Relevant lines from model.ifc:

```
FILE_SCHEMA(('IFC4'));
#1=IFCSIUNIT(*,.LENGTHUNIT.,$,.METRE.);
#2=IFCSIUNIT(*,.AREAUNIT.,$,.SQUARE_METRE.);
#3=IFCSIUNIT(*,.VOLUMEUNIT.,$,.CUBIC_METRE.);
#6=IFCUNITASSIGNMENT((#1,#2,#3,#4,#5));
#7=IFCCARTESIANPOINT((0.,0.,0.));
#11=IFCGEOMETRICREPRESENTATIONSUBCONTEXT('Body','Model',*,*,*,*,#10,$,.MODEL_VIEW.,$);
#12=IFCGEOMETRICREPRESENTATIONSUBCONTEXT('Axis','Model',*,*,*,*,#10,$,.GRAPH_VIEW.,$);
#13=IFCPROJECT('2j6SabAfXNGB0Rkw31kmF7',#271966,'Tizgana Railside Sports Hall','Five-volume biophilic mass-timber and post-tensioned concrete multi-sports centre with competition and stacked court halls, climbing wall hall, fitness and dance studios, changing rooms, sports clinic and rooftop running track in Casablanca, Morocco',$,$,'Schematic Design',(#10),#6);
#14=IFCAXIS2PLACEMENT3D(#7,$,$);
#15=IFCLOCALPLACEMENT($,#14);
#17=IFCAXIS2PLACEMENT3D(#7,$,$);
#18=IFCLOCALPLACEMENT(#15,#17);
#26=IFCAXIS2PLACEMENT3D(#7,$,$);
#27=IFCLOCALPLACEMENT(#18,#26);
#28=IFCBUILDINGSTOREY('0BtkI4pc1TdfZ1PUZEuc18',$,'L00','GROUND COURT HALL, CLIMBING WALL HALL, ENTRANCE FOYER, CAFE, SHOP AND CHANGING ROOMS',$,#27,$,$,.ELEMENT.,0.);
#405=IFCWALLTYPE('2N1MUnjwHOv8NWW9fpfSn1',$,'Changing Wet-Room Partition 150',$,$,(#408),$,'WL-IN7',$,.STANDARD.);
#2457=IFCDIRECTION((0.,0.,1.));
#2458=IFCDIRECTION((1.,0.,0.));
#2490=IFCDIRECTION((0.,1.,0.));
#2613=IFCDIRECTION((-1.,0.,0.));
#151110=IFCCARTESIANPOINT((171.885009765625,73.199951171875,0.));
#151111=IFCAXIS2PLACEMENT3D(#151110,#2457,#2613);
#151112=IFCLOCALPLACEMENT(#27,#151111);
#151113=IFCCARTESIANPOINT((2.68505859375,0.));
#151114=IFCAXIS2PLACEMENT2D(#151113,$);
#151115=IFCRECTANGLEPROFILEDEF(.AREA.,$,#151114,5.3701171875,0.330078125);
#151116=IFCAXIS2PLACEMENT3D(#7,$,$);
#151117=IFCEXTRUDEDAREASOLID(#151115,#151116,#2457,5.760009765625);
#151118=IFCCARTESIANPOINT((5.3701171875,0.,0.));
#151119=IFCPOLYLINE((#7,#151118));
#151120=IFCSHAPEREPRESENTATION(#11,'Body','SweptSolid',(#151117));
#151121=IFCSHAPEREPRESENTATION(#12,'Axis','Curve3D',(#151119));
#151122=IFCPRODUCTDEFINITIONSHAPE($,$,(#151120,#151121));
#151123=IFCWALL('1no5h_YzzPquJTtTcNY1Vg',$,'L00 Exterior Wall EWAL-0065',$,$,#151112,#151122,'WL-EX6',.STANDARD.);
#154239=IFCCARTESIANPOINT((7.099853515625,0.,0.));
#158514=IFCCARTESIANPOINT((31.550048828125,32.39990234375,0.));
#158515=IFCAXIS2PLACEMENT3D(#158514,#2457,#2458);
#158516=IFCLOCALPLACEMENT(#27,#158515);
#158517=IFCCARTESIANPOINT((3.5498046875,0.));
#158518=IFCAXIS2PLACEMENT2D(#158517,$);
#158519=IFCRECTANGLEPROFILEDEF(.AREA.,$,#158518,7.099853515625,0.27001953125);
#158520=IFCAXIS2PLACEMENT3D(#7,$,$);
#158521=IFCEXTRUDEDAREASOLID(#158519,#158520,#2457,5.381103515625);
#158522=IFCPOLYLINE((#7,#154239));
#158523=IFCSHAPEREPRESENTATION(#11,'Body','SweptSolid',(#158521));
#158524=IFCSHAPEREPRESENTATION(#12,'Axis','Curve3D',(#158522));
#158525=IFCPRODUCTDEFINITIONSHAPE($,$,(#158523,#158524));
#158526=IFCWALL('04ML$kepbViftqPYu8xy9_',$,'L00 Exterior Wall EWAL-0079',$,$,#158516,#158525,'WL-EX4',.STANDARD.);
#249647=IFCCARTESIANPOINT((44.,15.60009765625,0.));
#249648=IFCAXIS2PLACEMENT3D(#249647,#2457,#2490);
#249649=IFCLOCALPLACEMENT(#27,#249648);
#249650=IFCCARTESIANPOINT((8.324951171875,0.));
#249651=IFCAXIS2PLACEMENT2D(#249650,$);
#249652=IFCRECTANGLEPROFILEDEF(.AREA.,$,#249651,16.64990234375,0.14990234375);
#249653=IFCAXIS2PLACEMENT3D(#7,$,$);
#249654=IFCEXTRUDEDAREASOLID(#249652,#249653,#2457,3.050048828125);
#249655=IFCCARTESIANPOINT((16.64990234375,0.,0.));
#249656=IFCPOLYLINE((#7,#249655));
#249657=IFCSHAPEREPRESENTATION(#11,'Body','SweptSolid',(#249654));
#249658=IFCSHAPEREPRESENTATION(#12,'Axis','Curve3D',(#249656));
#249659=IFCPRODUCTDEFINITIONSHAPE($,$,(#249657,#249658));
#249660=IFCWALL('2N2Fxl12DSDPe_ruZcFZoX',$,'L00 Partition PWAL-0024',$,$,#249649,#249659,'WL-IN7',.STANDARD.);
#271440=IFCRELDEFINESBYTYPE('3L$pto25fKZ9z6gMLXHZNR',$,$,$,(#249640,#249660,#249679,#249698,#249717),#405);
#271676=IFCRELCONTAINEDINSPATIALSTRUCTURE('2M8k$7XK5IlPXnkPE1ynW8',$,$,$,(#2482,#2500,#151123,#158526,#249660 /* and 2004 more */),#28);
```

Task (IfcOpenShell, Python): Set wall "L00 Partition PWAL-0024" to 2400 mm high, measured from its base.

```python
import ifcopenshell
import ifcopenshell.geom
import ifcopenshell.util.representation
import ifcopenshell.util.shape
import ifcopenshell.util.unit

model = ifcopenshell.open("model.ifc")
unit_scale = ifcopenshell.util.unit.calculate_unit_scale(model)
settings = ifcopenshell.geom.settings()


def volume(element):
    """Net volume in cubic metres, openings subtracted."""
    shape = ifcopenshell.geom.create_shape(settings, element)
    return ifcopenshell.util.shape.get_volume(shape.geometry)


wall = model.by_guid("2N2Fxl12DSDPe_ruZcFZoX")
before = volume(wall)

body = ifcopenshell.util.representation.get_representation(wall, "Model", "Body")
solid = body.Items[0]
old_height = solid.Depth
solid.Depth = 2.4 / unit_scale
after = volume(wall)

print(f"height {old_height:g} -> {solid.Depth:g}, volume {before:.3f} -> {after:.3f} m3")

model.write("model_updated.ifc")
```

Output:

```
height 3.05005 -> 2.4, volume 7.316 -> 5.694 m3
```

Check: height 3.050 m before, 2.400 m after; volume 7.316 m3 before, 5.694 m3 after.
